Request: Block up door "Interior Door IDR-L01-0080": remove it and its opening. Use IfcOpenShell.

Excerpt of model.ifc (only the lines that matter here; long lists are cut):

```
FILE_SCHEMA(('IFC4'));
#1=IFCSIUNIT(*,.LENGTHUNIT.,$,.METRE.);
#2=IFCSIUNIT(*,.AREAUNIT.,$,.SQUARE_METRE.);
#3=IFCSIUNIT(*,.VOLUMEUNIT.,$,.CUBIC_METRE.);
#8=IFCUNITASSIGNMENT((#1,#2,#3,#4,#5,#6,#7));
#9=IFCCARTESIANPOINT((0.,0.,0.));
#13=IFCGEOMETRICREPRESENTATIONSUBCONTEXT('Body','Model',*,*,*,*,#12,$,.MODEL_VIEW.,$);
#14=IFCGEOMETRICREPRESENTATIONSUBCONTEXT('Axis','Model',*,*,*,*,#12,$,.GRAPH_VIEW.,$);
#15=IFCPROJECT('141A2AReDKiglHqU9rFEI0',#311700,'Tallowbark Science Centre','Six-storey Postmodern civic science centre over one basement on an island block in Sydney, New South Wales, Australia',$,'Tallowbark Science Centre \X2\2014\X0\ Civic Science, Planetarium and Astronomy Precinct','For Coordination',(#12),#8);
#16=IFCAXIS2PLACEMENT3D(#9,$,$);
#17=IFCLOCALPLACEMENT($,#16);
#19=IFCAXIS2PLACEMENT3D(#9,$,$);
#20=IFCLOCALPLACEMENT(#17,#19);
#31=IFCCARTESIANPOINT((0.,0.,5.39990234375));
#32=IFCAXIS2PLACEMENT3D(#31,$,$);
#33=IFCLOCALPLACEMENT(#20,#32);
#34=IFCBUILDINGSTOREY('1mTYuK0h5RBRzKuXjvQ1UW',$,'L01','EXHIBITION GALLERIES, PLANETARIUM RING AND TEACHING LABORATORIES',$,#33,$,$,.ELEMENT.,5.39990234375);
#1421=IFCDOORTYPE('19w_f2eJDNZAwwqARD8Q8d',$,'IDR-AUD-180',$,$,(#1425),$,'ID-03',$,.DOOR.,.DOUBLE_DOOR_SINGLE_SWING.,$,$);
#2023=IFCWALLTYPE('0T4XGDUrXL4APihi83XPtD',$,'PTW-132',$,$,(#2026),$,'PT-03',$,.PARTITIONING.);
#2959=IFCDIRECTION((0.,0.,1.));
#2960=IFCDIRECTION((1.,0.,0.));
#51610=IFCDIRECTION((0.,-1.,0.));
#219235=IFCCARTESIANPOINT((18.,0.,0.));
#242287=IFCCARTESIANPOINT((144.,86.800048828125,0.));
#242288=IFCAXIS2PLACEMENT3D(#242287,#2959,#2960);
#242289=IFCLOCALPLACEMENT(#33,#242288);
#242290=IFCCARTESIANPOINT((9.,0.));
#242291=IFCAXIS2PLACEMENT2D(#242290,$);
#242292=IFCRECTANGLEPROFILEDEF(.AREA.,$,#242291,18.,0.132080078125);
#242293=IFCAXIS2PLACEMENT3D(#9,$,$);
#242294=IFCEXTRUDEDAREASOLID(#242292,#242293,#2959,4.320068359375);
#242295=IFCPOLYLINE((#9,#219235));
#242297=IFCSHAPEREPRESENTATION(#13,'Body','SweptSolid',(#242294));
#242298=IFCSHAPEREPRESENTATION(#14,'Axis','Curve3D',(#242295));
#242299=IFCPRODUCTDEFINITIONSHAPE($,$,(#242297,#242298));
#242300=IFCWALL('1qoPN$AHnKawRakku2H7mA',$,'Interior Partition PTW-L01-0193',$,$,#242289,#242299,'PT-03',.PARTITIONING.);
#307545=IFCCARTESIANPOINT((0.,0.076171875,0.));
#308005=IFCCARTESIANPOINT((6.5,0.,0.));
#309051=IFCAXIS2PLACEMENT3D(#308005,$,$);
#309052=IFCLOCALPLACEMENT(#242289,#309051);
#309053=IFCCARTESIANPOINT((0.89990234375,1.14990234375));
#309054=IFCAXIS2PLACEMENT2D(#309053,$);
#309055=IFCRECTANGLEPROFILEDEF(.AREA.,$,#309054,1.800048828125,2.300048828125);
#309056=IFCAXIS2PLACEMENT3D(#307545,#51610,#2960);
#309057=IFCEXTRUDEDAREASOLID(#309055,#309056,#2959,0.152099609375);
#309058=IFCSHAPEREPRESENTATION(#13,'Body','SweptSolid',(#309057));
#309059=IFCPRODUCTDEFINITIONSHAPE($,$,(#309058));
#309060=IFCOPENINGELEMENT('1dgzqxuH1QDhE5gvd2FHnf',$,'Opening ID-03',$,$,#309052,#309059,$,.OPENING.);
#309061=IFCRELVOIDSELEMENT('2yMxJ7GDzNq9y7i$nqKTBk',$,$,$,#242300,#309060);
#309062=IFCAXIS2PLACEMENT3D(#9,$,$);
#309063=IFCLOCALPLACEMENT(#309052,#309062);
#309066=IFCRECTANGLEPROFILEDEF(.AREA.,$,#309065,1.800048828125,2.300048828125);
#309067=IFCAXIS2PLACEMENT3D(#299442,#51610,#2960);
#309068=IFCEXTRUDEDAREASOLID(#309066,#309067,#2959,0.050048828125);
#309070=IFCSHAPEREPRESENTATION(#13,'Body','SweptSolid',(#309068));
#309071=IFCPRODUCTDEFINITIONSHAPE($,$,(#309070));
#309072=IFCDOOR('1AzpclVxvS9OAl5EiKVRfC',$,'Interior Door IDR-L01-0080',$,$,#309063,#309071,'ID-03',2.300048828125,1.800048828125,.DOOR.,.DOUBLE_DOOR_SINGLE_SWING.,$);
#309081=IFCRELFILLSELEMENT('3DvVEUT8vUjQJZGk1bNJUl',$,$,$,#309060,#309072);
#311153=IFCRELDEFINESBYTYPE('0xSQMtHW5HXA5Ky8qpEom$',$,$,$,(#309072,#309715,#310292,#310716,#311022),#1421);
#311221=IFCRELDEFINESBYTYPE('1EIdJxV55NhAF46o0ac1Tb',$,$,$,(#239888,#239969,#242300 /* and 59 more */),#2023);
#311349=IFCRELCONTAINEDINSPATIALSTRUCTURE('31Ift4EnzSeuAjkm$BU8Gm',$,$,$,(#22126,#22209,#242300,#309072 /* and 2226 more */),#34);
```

```python
import ifcopenshell
import ifcopenshell.api.feature
import ifcopenshell.api.root
import ifcopenshell.geom
import ifcopenshell.util.shape

model = ifcopenshell.open("model.ifc")
settings = ifcopenshell.geom.settings()


def volume(element):
    """Net volume in cubic metres, openings subtracted."""
    shape = ifcopenshell.geom.create_shape(settings, element)
    return ifcopenshell.util.shape.get_volume(shape.geometry)


door = model.by_guid("1AzpclVxvS9OAl5EiKVRfC")
opening = door.FillsVoids[0].RelatingOpeningElement
wall = opening.VoidsElements[0].RelatingBuildingElement
before = volume(wall)

ifcopenshell.api.root.remove_product(model, product=door)
ifcopenshell.api.feature.remove_feature(model, feature=opening)

after = volume(wall)

print(f"wall volume {before:.3f} -> {after:.3f} m3")

model.write("model_rev.ifc")
```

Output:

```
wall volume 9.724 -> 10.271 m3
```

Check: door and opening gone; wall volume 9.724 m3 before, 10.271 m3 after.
